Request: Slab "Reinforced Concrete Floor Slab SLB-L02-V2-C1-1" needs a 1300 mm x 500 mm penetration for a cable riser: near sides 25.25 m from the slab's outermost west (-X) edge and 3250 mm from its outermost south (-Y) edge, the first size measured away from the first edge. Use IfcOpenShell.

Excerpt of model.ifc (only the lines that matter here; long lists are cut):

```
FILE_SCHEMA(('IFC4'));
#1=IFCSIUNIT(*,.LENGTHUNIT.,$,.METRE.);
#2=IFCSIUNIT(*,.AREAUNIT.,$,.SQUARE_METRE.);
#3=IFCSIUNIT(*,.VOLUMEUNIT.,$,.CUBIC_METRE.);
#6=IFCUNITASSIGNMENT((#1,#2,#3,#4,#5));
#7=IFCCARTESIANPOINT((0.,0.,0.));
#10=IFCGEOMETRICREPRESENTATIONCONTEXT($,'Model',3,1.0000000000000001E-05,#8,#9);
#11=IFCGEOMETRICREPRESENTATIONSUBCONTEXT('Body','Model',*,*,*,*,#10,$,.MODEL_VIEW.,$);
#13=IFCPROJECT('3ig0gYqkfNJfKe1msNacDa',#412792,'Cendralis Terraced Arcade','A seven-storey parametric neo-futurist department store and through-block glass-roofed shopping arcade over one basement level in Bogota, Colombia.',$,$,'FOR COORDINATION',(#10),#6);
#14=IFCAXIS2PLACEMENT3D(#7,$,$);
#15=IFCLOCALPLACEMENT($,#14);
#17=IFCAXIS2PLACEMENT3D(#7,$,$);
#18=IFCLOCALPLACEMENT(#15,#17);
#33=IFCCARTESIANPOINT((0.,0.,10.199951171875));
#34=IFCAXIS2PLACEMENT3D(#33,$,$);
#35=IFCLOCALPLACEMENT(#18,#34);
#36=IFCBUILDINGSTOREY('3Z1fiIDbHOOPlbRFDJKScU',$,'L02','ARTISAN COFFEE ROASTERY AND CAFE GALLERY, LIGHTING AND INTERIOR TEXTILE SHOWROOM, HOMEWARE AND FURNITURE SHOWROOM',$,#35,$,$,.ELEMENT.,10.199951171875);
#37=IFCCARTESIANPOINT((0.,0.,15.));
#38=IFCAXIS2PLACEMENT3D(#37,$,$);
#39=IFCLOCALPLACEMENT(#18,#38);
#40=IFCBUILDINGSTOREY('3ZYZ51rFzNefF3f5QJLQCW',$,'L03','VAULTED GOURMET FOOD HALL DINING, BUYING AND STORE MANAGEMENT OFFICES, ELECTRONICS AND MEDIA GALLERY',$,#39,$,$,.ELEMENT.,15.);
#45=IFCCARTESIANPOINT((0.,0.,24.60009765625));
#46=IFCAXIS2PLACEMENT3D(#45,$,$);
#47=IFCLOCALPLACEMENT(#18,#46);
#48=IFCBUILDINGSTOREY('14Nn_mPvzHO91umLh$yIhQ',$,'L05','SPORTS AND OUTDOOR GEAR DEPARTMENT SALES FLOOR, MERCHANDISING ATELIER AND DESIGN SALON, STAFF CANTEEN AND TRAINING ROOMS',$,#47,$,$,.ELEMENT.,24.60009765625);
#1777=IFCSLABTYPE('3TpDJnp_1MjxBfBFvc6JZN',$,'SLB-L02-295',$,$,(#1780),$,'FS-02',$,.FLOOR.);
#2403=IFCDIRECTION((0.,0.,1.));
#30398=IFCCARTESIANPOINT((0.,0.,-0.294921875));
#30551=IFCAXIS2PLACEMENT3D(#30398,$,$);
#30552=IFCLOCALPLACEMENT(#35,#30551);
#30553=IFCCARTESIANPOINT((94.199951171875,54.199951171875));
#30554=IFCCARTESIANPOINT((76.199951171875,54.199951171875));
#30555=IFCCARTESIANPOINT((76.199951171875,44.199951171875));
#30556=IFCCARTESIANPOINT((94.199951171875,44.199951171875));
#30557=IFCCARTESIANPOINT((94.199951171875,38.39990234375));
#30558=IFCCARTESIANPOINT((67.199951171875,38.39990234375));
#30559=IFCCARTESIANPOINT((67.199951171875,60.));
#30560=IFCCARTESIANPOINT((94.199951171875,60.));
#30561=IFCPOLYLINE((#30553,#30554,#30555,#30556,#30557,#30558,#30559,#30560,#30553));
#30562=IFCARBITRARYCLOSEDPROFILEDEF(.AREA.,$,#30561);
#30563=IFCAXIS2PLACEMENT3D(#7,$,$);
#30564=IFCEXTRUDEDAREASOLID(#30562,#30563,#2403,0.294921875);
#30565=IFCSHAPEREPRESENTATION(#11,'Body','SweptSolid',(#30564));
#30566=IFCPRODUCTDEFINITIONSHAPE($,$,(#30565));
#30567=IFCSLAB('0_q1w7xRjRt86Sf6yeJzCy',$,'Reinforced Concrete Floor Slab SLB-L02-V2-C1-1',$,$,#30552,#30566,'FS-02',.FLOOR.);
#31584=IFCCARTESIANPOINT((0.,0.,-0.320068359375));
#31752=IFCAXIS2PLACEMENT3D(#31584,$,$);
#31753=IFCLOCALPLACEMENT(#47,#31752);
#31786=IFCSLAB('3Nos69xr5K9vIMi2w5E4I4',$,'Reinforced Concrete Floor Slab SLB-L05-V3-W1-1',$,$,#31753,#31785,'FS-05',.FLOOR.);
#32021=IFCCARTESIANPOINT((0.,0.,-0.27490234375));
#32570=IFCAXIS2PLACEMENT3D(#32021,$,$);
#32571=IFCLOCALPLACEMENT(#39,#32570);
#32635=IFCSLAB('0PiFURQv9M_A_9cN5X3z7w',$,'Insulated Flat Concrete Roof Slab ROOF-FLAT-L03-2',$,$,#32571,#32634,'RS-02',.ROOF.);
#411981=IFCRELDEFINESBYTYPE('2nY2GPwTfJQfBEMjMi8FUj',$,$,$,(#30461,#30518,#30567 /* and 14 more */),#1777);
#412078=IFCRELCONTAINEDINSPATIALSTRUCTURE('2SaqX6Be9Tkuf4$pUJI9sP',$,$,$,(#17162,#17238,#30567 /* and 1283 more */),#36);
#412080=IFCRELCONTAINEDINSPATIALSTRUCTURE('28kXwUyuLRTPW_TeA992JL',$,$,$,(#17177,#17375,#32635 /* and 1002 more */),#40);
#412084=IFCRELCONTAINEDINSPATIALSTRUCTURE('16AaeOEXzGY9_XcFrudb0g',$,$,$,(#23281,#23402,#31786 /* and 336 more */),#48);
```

```python
import numpy as np
import ifcopenshell
import ifcopenshell.api.feature
import ifcopenshell.api.geometry
import ifcopenshell.api.root
import ifcopenshell.geom
import ifcopenshell.util.placement
import ifcopenshell.util.representation
import ifcopenshell.util.shape
import ifcopenshell.util.unit

model = ifcopenshell.open("model.ifc")
unit_scale = ifcopenshell.util.unit.calculate_unit_scale(model)
settings = ifcopenshell.geom.settings()


def volume(element):
    """Net volume in cubic metres, openings subtracted."""
    shape = ifcopenshell.geom.create_shape(settings, element)
    return ifcopenshell.util.shape.get_volume(shape.geometry)


slab = model.by_guid("0_q1w7xRjRt86Sf6yeJzCy")
before = volume(slab)

# Extent in the slab's own axes, in metres. The edges named are its -X and -Y sides.
slab_shape = ifcopenshell.geom.create_shape(settings, slab)
vertices = ifcopenshell.util.shape.get_vertices(slab_shape.geometry)
x_min, y_min, bottom = vertices.min(axis=0)
top = vertices[:, 2].max()

opening = ifcopenshell.api.root.create_entity(model, ifc_class="IfcOpeningElement", name="Cable riser opening", predefined_type="OPENING")
context = ifcopenshell.util.representation.get_context(model, "Model", "Body", "MODEL_VIEW")
width, depth = 1.3, 0.5
outline = [(0.0, 0.0), (width, 0.0), (width, depth), (0.0, depth), (0.0, 0.0)]
# Overshoot both faces by 50 mm so the cut is clean.
shape = ifcopenshell.api.geometry.add_slab_representation(
    model, context=context, depth=top - bottom + 0.1, polyline=outline
)
ifcopenshell.api.geometry.assign_representation(model, product=opening, representation=shape)

matrix = ifcopenshell.util.placement.get_local_placement(slab.ObjectPlacement)
matrix[:, 3] = matrix @ np.append(np.array([x_min + 25.25, y_min + 3.25, bottom - 0.05]) / unit_scale, 1.0)
ifcopenshell.api.geometry.edit_object_placement(model, product=opening, matrix=matrix, is_si=False)
ifcopenshell.api.feature.add_feature(model, feature=opening, element=slab)

after = volume(slab)

print(f"slab volume {before:.3f} -> {after:.3f} m3")

model.write("model_edited.ifc")
```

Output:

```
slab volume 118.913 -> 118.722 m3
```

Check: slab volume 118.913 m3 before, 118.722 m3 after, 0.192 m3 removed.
